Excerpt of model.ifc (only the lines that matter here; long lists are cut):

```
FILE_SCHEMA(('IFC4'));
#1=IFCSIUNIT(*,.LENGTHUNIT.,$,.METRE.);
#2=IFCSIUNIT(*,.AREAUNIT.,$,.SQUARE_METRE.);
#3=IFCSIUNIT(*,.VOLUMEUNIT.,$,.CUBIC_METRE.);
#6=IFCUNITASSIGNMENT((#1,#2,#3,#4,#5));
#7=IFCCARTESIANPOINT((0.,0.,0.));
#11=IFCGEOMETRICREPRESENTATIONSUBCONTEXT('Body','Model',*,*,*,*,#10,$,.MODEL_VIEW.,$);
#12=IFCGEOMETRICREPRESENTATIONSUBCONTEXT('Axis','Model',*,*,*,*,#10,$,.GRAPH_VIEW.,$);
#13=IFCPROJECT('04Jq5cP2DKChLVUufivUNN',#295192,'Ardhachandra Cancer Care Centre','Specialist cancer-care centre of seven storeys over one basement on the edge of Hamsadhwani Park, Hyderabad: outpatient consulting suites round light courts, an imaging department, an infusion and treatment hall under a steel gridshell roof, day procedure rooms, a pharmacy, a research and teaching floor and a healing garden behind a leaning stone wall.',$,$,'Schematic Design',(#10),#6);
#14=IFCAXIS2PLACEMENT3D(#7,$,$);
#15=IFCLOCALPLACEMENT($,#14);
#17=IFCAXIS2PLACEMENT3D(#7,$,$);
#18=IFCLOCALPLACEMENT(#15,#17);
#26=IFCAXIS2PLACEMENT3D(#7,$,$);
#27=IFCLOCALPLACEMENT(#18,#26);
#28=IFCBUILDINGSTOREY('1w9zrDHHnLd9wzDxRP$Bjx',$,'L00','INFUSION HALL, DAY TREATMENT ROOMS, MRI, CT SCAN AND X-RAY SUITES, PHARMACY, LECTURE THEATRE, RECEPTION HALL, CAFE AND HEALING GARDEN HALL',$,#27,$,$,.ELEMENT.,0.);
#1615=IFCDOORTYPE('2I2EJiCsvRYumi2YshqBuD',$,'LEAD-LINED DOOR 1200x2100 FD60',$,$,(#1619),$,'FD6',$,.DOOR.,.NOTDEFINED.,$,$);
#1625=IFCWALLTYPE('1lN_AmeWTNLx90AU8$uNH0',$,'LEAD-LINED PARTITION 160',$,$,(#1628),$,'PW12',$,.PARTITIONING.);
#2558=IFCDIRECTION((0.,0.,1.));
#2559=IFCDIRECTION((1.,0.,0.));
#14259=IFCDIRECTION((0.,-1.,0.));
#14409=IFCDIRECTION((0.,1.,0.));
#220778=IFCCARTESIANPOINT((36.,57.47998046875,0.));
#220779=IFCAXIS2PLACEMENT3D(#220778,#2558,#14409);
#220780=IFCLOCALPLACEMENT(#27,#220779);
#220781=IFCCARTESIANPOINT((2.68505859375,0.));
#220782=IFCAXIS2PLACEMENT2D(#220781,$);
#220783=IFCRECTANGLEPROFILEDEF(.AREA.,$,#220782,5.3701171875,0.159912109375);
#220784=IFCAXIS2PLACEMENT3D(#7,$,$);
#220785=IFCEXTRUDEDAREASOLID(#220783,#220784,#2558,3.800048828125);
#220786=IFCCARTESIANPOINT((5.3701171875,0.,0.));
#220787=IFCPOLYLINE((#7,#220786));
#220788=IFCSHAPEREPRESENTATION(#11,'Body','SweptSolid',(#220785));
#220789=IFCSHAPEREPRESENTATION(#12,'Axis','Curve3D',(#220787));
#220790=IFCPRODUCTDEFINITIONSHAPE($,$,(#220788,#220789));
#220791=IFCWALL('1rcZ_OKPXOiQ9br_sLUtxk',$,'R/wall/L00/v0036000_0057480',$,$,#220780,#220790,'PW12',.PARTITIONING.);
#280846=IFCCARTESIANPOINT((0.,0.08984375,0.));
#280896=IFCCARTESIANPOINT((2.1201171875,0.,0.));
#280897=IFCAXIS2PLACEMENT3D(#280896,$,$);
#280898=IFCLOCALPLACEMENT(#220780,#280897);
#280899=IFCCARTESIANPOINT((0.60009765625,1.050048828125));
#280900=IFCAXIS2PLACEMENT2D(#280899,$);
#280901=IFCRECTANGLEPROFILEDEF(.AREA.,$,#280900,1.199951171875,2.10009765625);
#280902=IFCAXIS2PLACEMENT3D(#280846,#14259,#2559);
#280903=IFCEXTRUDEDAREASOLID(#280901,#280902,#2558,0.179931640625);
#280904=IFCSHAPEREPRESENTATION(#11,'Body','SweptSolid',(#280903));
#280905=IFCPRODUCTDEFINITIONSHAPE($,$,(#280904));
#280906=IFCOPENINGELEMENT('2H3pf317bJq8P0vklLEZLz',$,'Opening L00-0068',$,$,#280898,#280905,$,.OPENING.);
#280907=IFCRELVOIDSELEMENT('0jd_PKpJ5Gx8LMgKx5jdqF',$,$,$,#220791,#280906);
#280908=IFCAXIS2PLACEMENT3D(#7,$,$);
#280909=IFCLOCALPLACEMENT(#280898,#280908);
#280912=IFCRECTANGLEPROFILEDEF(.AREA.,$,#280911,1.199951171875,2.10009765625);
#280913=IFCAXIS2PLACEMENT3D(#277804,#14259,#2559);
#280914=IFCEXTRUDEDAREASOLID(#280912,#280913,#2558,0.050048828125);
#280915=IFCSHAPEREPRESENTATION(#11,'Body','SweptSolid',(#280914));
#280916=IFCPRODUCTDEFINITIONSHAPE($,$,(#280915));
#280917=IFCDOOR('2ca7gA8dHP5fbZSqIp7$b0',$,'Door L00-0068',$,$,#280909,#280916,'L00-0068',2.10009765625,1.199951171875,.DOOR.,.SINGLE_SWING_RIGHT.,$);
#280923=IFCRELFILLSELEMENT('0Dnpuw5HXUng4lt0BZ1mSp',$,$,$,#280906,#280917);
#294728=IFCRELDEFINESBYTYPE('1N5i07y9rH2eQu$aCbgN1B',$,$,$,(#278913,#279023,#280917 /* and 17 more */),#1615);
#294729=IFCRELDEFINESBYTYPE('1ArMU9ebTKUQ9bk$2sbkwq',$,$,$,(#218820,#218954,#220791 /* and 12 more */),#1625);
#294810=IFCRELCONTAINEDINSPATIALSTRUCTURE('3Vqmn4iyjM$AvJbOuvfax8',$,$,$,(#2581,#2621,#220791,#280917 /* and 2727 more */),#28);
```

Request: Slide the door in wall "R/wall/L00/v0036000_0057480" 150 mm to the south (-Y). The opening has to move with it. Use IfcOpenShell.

```python
import ifcopenshell
import ifcopenshell.api.geometry
import ifcopenshell.util.placement
import ifcopenshell.util.unit

model = ifcopenshell.open("model.ifc")
unit_scale = ifcopenshell.util.unit.calculate_unit_scale(model)

door = model.by_guid("2ca7gA8dHP5fbZSqIp7$b0")
opening = door.FillsVoids[0].RelatingOpeningElement
wall = opening.VoidsElements[0].RelatingBuildingElement

wall_matrix = ifcopenshell.util.placement.get_local_placement(wall.ObjectPlacement)
shift = wall_matrix[:3, 0] * -0.15 / unit_scale
before = ifcopenshell.util.placement.get_local_placement(door.ObjectPlacement)[:3, 3].copy()

# The door is placed relative to its opening, so it follows when the opening moves.
matrix = ifcopenshell.util.placement.get_local_placement(opening.ObjectPlacement)
matrix[:3, 3] += shift
ifcopenshell.api.geometry.edit_object_placement(
    model, product=opening, matrix=matrix, is_si=False, should_transform_children=True
)

after = ifcopenshell.util.placement.get_local_placement(door.ObjectPlacement)[:3, 3]
print("door moved by", (after - before).round(3) + 0.0)

model.write("model_v2.ifc")
```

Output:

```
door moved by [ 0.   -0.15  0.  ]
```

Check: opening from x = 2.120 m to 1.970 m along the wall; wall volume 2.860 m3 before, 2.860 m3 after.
